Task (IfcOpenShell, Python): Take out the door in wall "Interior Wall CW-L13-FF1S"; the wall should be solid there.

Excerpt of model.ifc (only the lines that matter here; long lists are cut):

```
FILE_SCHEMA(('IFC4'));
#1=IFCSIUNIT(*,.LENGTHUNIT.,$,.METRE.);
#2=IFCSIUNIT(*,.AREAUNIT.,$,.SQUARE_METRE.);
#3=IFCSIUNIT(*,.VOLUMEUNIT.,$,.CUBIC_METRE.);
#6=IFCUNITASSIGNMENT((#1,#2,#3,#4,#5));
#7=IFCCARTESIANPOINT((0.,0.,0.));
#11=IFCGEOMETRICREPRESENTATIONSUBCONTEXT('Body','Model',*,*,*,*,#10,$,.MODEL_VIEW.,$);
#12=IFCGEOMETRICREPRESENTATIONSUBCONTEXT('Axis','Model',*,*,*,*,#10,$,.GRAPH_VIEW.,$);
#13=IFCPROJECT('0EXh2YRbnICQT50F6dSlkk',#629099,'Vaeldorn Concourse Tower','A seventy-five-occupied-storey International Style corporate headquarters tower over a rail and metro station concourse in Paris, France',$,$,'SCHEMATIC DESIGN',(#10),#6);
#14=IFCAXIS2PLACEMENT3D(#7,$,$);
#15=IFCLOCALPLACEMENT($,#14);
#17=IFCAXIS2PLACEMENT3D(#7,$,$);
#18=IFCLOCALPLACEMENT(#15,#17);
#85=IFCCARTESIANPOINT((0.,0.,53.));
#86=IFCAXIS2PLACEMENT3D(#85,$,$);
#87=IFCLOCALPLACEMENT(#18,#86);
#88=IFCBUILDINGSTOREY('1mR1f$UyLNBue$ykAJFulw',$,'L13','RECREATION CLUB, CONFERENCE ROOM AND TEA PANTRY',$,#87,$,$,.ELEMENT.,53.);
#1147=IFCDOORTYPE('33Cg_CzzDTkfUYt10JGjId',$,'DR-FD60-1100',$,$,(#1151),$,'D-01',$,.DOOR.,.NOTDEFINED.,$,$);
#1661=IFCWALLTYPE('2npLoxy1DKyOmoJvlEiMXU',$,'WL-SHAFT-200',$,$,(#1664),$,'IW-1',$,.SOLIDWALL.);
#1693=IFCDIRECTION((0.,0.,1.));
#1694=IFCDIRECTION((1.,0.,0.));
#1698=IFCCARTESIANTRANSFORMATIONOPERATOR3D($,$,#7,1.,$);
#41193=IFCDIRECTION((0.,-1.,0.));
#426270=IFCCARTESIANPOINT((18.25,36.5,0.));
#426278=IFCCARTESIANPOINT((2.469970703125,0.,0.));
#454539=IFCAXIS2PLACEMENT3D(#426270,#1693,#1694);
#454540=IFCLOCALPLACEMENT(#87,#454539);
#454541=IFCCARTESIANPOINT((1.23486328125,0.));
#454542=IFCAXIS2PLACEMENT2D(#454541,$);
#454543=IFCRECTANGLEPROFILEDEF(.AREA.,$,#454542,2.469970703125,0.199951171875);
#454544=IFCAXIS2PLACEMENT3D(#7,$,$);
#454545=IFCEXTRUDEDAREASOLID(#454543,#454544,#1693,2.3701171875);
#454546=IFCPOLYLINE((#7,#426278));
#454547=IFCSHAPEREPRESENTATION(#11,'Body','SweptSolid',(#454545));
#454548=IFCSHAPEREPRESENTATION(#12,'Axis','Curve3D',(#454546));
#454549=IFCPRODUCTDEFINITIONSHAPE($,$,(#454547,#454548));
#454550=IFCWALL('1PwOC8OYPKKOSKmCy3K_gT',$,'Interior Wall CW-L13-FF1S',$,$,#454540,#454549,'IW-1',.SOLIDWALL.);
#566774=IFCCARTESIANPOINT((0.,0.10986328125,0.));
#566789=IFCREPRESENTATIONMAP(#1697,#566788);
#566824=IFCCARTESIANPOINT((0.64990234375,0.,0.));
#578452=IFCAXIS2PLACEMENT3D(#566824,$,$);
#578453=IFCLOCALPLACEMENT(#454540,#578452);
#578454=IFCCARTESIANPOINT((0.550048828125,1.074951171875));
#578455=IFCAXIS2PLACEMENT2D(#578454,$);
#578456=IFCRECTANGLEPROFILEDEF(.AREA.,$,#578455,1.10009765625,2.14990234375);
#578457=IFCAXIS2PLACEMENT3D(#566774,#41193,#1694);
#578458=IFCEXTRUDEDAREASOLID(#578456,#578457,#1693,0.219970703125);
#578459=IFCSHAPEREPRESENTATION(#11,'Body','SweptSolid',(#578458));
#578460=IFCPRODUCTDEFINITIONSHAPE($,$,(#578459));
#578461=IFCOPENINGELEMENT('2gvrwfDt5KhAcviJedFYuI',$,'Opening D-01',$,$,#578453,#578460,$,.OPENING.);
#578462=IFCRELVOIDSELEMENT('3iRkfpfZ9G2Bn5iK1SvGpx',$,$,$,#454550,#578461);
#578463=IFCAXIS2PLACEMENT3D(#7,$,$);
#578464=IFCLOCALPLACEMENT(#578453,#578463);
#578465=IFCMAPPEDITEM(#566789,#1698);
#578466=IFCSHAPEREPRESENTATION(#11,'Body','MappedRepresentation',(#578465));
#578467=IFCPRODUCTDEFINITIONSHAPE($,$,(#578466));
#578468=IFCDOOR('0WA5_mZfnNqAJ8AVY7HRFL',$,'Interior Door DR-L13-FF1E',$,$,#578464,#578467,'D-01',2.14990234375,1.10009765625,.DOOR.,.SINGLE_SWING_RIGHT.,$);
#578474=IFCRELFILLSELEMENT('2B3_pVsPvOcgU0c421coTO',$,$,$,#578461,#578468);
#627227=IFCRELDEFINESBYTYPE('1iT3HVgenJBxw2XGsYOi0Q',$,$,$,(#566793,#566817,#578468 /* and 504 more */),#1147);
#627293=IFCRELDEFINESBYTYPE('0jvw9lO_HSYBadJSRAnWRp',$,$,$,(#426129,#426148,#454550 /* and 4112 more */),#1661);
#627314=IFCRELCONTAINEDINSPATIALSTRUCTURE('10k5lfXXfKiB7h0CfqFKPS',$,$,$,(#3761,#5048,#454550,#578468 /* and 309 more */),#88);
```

```python
import ifcopenshell
import ifcopenshell.api.feature
import ifcopenshell.api.root
import ifcopenshell.geom
import ifcopenshell.util.shape

model = ifcopenshell.open("model.ifc")
settings = ifcopenshell.geom.settings()


def volume(element):
    """Net volume in cubic metres, openings subtracted."""
    shape = ifcopenshell.geom.create_shape(settings, element)
    return ifcopenshell.util.shape.get_volume(shape.geometry)


door = model.by_id(578468)
opening = door.FillsVoids[0].RelatingOpeningElement
wall = opening.VoidsElements[0].RelatingBuildingElement
before = volume(wall)

ifcopenshell.api.root.remove_product(model, product=door)
ifcopenshell.api.feature.remove_feature(model, feature=opening)

after = volume(wall)

print(f"wall volume {before:.3f} -> {after:.3f} m3")

model.write("model-out.ifc")
```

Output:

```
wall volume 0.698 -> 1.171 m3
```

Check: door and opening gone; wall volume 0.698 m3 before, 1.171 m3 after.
